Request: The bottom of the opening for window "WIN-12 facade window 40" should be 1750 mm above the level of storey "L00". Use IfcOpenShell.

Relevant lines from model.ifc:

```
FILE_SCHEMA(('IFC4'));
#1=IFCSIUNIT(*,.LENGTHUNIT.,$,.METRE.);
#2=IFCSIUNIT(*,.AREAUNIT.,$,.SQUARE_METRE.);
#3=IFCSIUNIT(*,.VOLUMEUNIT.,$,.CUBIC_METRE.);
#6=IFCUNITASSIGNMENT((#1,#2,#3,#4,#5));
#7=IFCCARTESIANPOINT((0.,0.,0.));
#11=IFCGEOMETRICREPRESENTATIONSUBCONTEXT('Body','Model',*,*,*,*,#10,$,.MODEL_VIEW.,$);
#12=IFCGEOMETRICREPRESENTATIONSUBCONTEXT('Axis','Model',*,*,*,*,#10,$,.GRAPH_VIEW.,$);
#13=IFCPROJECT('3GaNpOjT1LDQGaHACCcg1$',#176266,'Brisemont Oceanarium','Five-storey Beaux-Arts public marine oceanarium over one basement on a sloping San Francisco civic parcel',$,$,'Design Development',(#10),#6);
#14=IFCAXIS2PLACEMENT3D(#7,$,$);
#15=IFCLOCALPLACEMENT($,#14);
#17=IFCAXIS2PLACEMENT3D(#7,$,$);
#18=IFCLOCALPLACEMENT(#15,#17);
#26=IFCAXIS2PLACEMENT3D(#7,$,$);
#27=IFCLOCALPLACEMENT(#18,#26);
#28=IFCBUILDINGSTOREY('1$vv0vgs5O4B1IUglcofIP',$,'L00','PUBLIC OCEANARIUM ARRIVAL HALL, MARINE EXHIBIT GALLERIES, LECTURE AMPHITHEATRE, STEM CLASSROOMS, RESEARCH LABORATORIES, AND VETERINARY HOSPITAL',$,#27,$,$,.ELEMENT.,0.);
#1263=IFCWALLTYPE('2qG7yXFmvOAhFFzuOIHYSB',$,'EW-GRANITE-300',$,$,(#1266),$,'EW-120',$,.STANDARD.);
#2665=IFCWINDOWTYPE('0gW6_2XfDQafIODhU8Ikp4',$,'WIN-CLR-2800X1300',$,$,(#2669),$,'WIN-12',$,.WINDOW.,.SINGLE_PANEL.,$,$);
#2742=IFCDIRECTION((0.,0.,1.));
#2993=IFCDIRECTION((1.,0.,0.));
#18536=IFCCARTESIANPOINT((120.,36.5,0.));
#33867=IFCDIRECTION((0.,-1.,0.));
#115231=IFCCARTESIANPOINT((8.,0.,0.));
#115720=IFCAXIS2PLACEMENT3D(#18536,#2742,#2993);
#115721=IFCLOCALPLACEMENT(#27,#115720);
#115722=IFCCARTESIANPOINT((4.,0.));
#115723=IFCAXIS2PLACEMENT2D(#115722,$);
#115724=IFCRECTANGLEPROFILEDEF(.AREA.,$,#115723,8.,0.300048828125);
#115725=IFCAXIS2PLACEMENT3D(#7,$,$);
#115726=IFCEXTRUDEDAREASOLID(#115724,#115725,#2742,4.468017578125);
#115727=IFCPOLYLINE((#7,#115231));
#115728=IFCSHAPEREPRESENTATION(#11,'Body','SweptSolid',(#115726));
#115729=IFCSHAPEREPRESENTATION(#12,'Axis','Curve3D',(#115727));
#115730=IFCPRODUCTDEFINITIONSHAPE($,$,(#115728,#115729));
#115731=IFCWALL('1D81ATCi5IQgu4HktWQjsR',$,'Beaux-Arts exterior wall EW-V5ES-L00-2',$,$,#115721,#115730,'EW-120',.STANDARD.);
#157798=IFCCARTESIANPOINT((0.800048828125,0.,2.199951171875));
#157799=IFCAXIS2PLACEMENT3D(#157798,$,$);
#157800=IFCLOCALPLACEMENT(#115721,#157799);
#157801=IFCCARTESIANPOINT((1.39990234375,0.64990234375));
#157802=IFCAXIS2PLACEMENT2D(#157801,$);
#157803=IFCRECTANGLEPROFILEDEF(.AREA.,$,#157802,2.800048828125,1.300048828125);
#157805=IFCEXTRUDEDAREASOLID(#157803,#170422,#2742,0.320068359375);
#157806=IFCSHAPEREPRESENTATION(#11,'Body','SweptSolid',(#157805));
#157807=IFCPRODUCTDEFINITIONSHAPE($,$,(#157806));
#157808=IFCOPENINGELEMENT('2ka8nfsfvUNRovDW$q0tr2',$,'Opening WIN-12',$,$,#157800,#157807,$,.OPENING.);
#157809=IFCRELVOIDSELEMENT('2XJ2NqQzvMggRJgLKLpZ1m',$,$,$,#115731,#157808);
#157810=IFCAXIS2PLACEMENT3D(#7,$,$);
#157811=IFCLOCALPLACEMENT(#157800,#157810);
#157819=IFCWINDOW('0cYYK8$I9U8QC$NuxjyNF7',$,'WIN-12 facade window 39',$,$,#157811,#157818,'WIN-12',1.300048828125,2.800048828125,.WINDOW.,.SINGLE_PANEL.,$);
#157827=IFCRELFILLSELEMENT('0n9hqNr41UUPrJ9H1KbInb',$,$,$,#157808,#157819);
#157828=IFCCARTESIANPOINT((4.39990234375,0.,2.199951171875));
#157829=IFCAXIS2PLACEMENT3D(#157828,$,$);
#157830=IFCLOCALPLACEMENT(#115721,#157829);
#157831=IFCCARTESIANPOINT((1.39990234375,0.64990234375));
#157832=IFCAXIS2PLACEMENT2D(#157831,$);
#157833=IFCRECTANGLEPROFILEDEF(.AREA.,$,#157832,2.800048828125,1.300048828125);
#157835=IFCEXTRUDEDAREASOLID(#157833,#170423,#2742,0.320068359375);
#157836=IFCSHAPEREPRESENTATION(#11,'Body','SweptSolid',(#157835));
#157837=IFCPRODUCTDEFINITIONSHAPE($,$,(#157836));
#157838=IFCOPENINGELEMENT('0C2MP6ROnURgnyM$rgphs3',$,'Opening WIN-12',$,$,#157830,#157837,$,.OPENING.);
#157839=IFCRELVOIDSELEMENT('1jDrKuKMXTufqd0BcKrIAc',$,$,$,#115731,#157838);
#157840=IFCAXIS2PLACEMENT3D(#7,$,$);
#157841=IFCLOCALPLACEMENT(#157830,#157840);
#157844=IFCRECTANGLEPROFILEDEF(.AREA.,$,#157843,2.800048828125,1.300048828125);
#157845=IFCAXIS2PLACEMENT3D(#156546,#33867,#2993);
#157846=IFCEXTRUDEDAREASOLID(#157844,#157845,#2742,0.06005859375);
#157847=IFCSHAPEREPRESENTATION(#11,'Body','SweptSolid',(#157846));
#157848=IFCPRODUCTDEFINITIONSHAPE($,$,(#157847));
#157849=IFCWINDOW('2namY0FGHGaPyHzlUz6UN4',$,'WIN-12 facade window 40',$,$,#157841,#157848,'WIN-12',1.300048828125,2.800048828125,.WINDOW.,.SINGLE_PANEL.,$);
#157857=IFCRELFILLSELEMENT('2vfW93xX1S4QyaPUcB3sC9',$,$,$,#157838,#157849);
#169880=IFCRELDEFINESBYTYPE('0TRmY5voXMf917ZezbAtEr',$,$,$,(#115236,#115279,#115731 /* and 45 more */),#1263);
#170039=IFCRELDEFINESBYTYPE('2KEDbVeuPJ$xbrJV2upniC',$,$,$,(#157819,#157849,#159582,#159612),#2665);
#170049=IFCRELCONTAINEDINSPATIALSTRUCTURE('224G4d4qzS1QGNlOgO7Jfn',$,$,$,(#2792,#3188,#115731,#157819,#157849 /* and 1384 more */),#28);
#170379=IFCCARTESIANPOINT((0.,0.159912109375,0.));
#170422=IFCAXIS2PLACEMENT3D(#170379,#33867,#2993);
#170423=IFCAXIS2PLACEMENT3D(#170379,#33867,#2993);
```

```python
import numpy as np
import ifcopenshell
import ifcopenshell.api.geometry
import ifcopenshell.geom
import ifcopenshell.util.element
import ifcopenshell.util.placement
import ifcopenshell.util.shape
import ifcopenshell.util.unit

model = ifcopenshell.open("model.ifc")
unit_scale = ifcopenshell.util.unit.calculate_unit_scale(model)

window = model.by_guid("2namY0FGHGaPyHzlUz6UN4")
opening = window.FillsVoids[0].RelatingOpeningElement
storey = ifcopenshell.util.element.get_container(window, ifc_class="IfcBuildingStorey")
level = ifcopenshell.util.placement.get_local_placement(storey.ObjectPlacement)[2, 3]

# The opening's origin need not be at the sill, so measure its lowest point.
shape = ifcopenshell.geom.create_shape(ifcopenshell.geom.settings(), opening)
bottom = ifcopenshell.util.shape.get_shape_bottom_elevation(shape, shape.geometry) / unit_scale
dz = level + 1.75 - bottom

shift = np.array([0.0, 0.0, dz])
# The window is placed relative to its opening, so it follows when the opening moves.
matrix = ifcopenshell.util.placement.get_local_placement(opening.ObjectPlacement)
matrix[:3, 3] += shift
ifcopenshell.api.geometry.edit_object_placement(
    model, product=opening, matrix=matrix, is_si=False, should_transform_children=True
)

print(f"moved by {dz * unit_scale:+.3f} m")

model.write("model_v2.ifc")
```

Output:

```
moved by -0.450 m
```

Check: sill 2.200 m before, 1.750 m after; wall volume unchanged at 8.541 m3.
